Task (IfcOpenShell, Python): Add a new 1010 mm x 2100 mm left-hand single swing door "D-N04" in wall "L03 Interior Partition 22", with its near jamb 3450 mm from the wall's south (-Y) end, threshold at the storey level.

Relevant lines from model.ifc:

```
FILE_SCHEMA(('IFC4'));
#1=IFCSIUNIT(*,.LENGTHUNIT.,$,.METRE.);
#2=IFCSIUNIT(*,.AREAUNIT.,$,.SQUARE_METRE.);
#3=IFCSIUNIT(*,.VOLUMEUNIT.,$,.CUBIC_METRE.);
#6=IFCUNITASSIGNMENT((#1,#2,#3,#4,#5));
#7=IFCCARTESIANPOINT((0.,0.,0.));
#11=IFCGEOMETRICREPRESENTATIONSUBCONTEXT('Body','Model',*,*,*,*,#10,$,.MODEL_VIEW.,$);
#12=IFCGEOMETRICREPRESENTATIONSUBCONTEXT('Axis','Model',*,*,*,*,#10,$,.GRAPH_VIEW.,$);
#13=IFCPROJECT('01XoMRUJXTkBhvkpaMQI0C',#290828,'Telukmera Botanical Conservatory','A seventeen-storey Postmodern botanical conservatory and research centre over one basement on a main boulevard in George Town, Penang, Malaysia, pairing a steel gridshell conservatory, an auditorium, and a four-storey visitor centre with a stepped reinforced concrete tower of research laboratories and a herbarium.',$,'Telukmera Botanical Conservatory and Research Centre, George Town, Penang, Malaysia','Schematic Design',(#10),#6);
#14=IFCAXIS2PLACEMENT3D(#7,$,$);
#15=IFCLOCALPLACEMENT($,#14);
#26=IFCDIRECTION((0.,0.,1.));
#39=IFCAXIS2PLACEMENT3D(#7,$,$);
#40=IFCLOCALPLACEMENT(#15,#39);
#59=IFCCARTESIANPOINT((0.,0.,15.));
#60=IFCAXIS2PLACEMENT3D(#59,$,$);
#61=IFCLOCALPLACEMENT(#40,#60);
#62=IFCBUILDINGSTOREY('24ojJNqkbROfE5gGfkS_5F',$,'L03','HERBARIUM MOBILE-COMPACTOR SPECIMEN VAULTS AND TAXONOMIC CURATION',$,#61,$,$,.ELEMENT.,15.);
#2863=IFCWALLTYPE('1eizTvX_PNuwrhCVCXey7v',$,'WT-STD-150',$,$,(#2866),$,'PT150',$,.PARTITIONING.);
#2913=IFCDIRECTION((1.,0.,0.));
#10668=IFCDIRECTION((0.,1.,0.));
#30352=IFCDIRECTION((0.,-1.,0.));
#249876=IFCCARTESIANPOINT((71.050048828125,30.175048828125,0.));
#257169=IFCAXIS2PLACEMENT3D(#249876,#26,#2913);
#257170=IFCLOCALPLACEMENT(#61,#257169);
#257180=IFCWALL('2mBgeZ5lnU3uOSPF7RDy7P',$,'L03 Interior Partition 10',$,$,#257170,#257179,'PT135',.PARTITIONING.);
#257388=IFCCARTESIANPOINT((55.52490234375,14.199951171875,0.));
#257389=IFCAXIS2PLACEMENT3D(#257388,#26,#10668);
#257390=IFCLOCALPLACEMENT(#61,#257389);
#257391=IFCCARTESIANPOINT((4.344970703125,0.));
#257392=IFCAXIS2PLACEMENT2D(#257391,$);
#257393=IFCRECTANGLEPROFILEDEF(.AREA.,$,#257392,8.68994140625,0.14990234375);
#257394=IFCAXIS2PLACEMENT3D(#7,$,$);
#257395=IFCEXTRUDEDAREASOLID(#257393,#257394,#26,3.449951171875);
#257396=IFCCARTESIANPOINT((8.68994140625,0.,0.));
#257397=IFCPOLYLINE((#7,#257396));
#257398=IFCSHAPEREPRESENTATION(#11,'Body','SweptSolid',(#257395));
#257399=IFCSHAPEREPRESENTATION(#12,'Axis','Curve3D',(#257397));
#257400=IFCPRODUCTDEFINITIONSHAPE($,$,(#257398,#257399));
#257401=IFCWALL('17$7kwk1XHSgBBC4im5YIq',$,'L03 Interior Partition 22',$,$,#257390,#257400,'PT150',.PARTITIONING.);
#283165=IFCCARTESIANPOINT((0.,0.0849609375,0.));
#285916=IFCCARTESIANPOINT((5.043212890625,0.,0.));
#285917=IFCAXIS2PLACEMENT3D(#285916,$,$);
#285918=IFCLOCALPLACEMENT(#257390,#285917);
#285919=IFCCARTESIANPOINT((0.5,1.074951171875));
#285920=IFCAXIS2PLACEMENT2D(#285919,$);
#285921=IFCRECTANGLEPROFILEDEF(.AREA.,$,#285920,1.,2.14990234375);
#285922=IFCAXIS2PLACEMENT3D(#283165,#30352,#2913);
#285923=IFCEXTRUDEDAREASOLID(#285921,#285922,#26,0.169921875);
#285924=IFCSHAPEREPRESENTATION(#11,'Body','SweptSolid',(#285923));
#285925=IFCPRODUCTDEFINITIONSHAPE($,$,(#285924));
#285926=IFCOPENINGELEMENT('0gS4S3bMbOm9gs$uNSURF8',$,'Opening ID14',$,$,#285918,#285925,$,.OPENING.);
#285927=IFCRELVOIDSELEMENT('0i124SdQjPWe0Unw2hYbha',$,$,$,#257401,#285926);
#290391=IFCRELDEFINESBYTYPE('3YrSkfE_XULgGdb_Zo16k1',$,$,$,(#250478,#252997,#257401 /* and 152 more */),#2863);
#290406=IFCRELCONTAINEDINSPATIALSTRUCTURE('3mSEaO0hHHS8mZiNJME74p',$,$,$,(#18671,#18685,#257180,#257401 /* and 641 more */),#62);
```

```python
import numpy as np
import ifcopenshell
import ifcopenshell.api.feature
import ifcopenshell.api.geometry
import ifcopenshell.api.root
import ifcopenshell.api.spatial
import ifcopenshell.geom
import ifcopenshell.util.element
import ifcopenshell.util.placement
import ifcopenshell.util.representation
import ifcopenshell.util.shape
import ifcopenshell.util.unit

model = ifcopenshell.open("model.ifc")
unit_scale = ifcopenshell.util.unit.calculate_unit_scale(model)
settings = ifcopenshell.geom.settings()


def volume(element):
    """Net volume in cubic metres, openings subtracted."""
    shape = ifcopenshell.geom.create_shape(settings, element)
    return ifcopenshell.util.shape.get_volume(shape.geometry)


wall = model.by_guid("17$7kwk1XHSgBBC4im5YIq")
storey = ifcopenshell.util.element.get_container(wall, ifc_class="IfcBuildingStorey")
context = ifcopenshell.util.representation.get_context(model, "Model", "Body", "MODEL_VIEW")
before = volume(wall)

width, height, from_end, sill = 1.01, 2.1, 3.45, 0.0  # metres

# The wall runs along its own X axis, and the end named is its -X end.
wall_shape = ifcopenshell.geom.create_shape(settings, wall)
x, y, z = ifcopenshell.util.shape.get_vertices(wall_shape.geometry).T
start = x.min() + from_end
face, thickness = float(y.min()), float(y.max() - y.min())
wall_matrix = ifcopenshell.util.placement.get_local_placement(wall.ObjectPlacement)
level = ifcopenshell.util.placement.get_local_placement(storey.ObjectPlacement)[2, 3]


def in_wall(x, y):
    """Placement at x, y metres in the wall's axes, at sill height."""
    matrix = wall_matrix.copy()
    matrix[:, 3] = wall_matrix @ np.array([x / unit_scale, y / unit_scale, 0.0, 1.0])
    matrix[2, 3] = level + sill / unit_scale
    return matrix


# Opening: a box that overshoots both wall faces by 50 mm.
opening = ifcopenshell.api.root.create_entity(model, ifc_class="IfcOpeningElement", predefined_type="OPENING")
box = ifcopenshell.api.geometry.add_wall_representation(
    model, context=context, length=width, height=height, thickness=thickness + 0.1
)
ifcopenshell.api.geometry.assign_representation(model, product=opening, representation=box)
ifcopenshell.api.geometry.edit_object_placement(model, product=opening, matrix=in_wall(start, face - 0.05), is_si=False)
ifcopenshell.api.feature.add_feature(model, feature=opening, element=wall)

door = ifcopenshell.api.root.create_entity(model, ifc_class="IfcDoor", name="D-N04", predefined_type="DOOR")
door.OverallWidth, door.OverallHeight = width / unit_scale, height / unit_scale
door.OperationType = "SINGLE_SWING_LEFT"
body = ifcopenshell.api.geometry.add_door_representation(
    model,
    context=context,
    overall_width=door.OverallWidth,
    overall_height=door.OverallHeight,
    operation_type="SINGLE_SWING_LEFT",
    lining_properties={"LiningDepth": thickness / unit_scale, "ThresholdDepth": thickness / unit_scale},
)
ifcopenshell.api.geometry.assign_representation(model, product=door, representation=body)
ifcopenshell.api.spatial.assign_container(model, products=[door], relating_structure=storey)
ifcopenshell.api.feature.add_filling(model, opening=opening, element=door)

# The lining spans the wall, so the door starts at the wall face.
ifcopenshell.api.geometry.edit_object_placement(model, product=door, matrix=in_wall(start, face), is_si=False)

after = volume(wall)

print(f"wall volume {before:.3f} -> {after:.3f} m3")

model.write("model-out.ifc")
```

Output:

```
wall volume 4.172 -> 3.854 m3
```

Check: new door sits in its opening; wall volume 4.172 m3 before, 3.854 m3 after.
